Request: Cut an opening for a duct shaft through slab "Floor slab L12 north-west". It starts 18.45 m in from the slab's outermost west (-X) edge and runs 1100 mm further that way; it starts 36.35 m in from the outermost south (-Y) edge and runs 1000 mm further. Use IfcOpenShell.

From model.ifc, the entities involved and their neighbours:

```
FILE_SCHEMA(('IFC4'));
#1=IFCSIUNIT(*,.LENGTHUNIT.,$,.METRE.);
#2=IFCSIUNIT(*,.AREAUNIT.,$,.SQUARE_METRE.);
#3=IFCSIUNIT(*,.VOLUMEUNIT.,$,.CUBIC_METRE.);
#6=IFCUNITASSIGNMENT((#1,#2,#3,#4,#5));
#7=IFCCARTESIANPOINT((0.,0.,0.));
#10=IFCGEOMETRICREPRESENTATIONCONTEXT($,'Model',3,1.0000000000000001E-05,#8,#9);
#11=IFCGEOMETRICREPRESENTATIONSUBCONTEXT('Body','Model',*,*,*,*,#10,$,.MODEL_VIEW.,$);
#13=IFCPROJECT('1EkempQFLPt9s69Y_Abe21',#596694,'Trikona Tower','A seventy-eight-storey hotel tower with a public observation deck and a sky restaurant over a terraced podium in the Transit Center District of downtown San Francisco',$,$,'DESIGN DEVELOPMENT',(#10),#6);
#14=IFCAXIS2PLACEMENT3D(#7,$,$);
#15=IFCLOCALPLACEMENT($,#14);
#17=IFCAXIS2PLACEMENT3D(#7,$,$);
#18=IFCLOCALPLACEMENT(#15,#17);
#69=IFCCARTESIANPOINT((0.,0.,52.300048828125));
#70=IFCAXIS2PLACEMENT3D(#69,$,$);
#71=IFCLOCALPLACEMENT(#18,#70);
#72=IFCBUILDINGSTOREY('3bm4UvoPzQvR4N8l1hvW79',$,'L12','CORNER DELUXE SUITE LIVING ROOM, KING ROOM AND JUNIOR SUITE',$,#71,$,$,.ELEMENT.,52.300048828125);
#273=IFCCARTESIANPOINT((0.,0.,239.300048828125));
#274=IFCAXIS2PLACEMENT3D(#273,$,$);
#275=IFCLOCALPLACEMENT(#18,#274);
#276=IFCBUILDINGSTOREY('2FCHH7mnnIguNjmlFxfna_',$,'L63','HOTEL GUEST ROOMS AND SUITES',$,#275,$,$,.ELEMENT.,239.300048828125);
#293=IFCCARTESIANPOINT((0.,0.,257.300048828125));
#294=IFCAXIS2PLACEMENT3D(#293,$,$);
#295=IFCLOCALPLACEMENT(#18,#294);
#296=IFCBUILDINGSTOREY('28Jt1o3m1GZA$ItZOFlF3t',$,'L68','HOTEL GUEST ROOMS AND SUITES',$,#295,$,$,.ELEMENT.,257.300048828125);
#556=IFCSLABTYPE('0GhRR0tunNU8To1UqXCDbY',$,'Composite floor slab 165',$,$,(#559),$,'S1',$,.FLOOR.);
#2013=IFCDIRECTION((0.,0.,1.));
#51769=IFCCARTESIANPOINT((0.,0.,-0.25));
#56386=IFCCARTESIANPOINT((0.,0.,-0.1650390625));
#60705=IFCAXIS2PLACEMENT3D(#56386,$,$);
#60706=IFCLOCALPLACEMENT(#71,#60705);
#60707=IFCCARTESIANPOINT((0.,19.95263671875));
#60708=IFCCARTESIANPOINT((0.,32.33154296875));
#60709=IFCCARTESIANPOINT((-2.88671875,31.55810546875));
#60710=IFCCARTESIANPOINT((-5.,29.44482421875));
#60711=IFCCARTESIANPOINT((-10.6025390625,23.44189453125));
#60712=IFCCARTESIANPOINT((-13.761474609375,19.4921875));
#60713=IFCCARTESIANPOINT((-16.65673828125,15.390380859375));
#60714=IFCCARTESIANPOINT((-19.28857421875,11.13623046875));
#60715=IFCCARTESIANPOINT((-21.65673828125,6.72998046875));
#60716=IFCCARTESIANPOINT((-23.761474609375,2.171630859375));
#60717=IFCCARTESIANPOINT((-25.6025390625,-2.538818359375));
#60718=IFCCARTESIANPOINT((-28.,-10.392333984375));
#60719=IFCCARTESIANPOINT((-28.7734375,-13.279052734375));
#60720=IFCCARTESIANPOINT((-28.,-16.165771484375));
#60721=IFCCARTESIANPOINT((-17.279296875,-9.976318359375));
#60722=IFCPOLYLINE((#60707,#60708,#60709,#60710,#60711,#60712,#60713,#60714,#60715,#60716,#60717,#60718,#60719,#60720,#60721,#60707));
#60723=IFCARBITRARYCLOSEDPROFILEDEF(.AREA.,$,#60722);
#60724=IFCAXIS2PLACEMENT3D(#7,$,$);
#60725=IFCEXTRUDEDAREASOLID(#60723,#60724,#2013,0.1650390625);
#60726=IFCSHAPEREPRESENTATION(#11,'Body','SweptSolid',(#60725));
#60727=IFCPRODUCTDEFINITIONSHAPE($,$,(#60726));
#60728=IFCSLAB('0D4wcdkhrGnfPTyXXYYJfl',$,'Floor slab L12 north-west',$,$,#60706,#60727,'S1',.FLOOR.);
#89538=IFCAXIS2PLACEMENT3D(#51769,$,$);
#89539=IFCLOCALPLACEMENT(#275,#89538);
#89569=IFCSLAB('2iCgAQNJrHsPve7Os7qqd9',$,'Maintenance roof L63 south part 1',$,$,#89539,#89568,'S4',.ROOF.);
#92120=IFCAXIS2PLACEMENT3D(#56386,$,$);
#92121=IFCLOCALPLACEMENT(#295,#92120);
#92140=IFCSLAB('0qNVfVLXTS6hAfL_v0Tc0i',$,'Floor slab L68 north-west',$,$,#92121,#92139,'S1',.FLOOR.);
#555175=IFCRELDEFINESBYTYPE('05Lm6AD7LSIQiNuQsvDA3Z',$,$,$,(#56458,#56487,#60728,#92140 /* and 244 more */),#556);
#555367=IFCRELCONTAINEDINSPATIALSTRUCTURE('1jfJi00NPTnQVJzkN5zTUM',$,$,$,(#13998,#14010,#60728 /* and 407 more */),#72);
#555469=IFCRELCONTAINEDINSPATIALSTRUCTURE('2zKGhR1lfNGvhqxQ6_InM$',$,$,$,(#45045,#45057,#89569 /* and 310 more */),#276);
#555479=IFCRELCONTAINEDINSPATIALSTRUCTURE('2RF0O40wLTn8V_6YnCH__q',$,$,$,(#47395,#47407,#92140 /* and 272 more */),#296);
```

```python
import numpy as np
import ifcopenshell
import ifcopenshell.api.feature
import ifcopenshell.api.geometry
import ifcopenshell.api.root
import ifcopenshell.geom
import ifcopenshell.util.placement
import ifcopenshell.util.representation
import ifcopenshell.util.shape
import ifcopenshell.util.unit

model = ifcopenshell.open("model.ifc")
unit_scale = ifcopenshell.util.unit.calculate_unit_scale(model)
settings = ifcopenshell.geom.settings()


def volume(element):
    """Net volume in cubic metres, openings subtracted."""
    shape = ifcopenshell.geom.create_shape(settings, element)
    return ifcopenshell.util.shape.get_volume(shape.geometry)


slab = model.by_guid("0D4wcdkhrGnfPTyXXYYJfl")
before = volume(slab)

# Extent in the slab's own axes, in metres. The edges named are its -X and -Y sides.
slab_shape = ifcopenshell.geom.create_shape(settings, slab)
vertices = ifcopenshell.util.shape.get_vertices(slab_shape.geometry)
x_min, y_min, bottom = vertices.min(axis=0)
top = vertices[:, 2].max()

opening = ifcopenshell.api.root.create_entity(model, ifc_class="IfcOpeningElement", name="Duct shaft opening", predefined_type="OPENING")
context = ifcopenshell.util.representation.get_context(model, "Model", "Body", "MODEL_VIEW")
width, depth = 1.1, 1
outline = [(0.0, 0.0), (width, 0.0), (width, depth), (0.0, depth), (0.0, 0.0)]
# Overshoot both faces by 50 mm so the cut is clean.
shape = ifcopenshell.api.geometry.add_slab_representation(
    model, context=context, depth=top - bottom + 0.1, polyline=outline
)
ifcopenshell.api.geometry.assign_representation(model, product=opening, representation=shape)

matrix = ifcopenshell.util.placement.get_local_placement(slab.ObjectPlacement)
matrix[:, 3] = matrix @ np.append(np.array([x_min + 18.45, y_min + 36.35, bottom - 0.05]) / unit_scale, 1.0)
ifcopenshell.api.geometry.edit_object_placement(model, product=opening, matrix=matrix, is_si=False)
ifcopenshell.api.feature.add_feature(model, feature=opening, element=slab)

after = volume(slab)

print(f"slab volume {before:.3f} -> {after:.3f} m3")

model.write("model_edited.ifc")
```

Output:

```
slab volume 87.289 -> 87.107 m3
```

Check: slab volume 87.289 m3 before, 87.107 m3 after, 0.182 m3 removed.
